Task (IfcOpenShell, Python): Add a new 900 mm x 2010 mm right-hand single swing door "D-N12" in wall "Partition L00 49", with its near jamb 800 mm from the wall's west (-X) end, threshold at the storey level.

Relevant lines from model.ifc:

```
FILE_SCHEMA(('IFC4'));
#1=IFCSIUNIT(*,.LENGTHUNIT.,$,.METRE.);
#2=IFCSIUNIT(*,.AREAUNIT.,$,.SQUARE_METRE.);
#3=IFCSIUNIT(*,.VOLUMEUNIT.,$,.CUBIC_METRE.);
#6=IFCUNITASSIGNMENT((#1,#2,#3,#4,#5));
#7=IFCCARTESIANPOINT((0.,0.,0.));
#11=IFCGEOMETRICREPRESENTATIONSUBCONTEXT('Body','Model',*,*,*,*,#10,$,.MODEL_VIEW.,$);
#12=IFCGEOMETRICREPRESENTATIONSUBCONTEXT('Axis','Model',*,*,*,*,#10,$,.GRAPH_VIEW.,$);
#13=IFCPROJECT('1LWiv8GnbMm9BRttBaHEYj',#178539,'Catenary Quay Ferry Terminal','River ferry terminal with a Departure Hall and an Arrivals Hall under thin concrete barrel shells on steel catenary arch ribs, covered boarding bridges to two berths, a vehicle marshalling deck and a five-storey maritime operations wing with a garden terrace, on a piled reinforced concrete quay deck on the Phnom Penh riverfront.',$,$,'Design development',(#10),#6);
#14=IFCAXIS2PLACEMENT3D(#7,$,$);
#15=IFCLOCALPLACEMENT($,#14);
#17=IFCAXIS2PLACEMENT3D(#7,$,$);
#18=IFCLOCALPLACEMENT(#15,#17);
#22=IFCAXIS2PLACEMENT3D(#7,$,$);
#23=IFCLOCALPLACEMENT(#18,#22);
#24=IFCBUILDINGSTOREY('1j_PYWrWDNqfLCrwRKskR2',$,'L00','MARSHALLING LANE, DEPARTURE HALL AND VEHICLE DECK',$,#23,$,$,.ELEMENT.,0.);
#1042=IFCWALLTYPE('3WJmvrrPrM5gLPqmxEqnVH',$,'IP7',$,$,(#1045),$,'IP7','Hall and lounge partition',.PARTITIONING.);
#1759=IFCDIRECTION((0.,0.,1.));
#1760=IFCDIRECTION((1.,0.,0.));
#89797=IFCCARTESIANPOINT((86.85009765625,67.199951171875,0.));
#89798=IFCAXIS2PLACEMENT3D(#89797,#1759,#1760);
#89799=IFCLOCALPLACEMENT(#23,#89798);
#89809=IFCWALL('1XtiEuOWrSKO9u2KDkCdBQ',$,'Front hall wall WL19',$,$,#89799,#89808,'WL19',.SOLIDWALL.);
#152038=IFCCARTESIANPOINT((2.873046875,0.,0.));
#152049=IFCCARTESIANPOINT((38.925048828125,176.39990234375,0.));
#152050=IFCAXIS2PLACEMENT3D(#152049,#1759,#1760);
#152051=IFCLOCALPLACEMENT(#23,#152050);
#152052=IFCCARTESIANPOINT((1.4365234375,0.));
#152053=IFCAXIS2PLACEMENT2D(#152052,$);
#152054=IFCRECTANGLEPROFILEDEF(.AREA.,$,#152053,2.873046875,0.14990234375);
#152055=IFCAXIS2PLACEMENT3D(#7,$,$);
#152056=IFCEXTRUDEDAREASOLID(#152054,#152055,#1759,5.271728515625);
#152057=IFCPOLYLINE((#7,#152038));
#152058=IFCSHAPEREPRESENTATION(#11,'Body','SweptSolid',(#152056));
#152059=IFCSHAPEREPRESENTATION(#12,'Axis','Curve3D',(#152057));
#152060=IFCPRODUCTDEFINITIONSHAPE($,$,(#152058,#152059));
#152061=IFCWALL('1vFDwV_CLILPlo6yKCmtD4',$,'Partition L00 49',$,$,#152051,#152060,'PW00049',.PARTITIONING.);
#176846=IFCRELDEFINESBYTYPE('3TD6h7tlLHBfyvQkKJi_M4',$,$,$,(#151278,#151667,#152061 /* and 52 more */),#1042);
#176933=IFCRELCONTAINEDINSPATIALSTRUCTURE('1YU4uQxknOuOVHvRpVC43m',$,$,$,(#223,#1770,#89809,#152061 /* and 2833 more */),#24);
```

```python
import numpy as np
import ifcopenshell
import ifcopenshell.api.feature
import ifcopenshell.api.geometry
import ifcopenshell.api.root
import ifcopenshell.api.spatial
import ifcopenshell.geom
import ifcopenshell.util.element
import ifcopenshell.util.placement
import ifcopenshell.util.representation
import ifcopenshell.util.shape
import ifcopenshell.util.unit

model = ifcopenshell.open("model.ifc")
unit_scale = ifcopenshell.util.unit.calculate_unit_scale(model)
settings = ifcopenshell.geom.settings()


def volume(element):
    """Net volume in cubic metres, openings subtracted."""
    shape = ifcopenshell.geom.create_shape(settings, element)
    return ifcopenshell.util.shape.get_volume(shape.geometry)


wall = model.by_guid("1vFDwV_CLILPlo6yKCmtD4")
storey = ifcopenshell.util.element.get_container(wall, ifc_class="IfcBuildingStorey")
context = ifcopenshell.util.representation.get_context(model, "Model", "Body", "MODEL_VIEW")
before = volume(wall)

width, height, from_end, sill = 0.9, 2.01, 0.8, 0.0  # metres

# The wall runs along its own X axis, and the end named is its -X end.
wall_shape = ifcopenshell.geom.create_shape(settings, wall)
x, y, z = ifcopenshell.util.shape.get_vertices(wall_shape.geometry).T
start = x.min() + from_end
face, thickness = float(y.min()), float(y.max() - y.min())
wall_matrix = ifcopenshell.util.placement.get_local_placement(wall.ObjectPlacement)
level = ifcopenshell.util.placement.get_local_placement(storey.ObjectPlacement)[2, 3]


def in_wall(x, y):
    """Placement at x, y metres in the wall's axes, at sill height."""
    matrix = wall_matrix.copy()
    matrix[:, 3] = wall_matrix @ np.array([x / unit_scale, y / unit_scale, 0.0, 1.0])
    matrix[2, 3] = level + sill / unit_scale
    return matrix


# Opening: a box that overshoots both wall faces by 50 mm.
opening = ifcopenshell.api.root.create_entity(model, ifc_class="IfcOpeningElement", predefined_type="OPENING")
box = ifcopenshell.api.geometry.add_wall_representation(
    model, context=context, length=width, height=height, thickness=thickness + 0.1
)
ifcopenshell.api.geometry.assign_representation(model, product=opening, representation=box)
ifcopenshell.api.geometry.edit_object_placement(model, product=opening, matrix=in_wall(start, face - 0.05), is_si=False)
ifcopenshell.api.feature.add_feature(model, feature=opening, element=wall)

door = ifcopenshell.api.root.create_entity(model, ifc_class="IfcDoor", name="D-N12", predefined_type="DOOR")
door.OverallWidth, door.OverallHeight = width / unit_scale, height / unit_scale
door.OperationType = "SINGLE_SWING_RIGHT"
body = ifcopenshell.api.geometry.add_door_representation(
    model,
    context=context,
    overall_width=door.OverallWidth,
    overall_height=door.OverallHeight,
    operation_type="SINGLE_SWING_RIGHT",
    lining_properties={"LiningDepth": thickness / unit_scale, "ThresholdDepth": thickness / unit_scale},
)
ifcopenshell.api.geometry.assign_representation(model, product=door, representation=body)
ifcopenshell.api.spatial.assign_container(model, products=[door], relating_structure=storey)
ifcopenshell.api.feature.add_filling(model, opening=opening, element=door)

# The lining spans the wall, so the door starts at the wall face.
ifcopenshell.api.geometry.edit_object_placement(model, product=door, matrix=in_wall(start, face), is_si=False)

after = volume(wall)

print(f"wall volume {before:.3f} -> {after:.3f} m3")

model.write("model_rev.ifc")
```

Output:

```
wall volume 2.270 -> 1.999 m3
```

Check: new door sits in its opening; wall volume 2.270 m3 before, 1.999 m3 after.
